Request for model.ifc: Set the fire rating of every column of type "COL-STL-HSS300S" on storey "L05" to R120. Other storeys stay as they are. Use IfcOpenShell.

First a look at what the model holds.

```python
import ifcopenshell
import ifcopenshell.util.element

model = ifcopenshell.open("model.ifc")
print(model.schema)
storey = next(s for s in model.by_type("IfcBuildingStorey") if s.Name == "L05")
columns = [e for e in ifcopenshell.util.element.get_decomposition(storey) if e.is_a("IfcColumn")]
seen = {}
for e in columns:
    element_type = ifcopenshell.util.element.get_type(e)
    key = (element_type.Name if element_type != e and element_type else None, ifcopenshell.util.element.get_pset(e, "Pset_ColumnCommon", "FireRating"))
    seen[key] = seen.get(key, 0) + 1
for (name, value), count in sorted(seen.items(), key=str):
    print(count, "x", name, "|", value)
```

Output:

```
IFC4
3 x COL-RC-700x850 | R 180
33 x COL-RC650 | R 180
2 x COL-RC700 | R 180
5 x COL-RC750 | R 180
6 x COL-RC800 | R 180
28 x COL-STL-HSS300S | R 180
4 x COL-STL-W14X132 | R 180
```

```python
import ifcopenshell
import ifcopenshell.api.pset
import ifcopenshell.util.element

model = ifcopenshell.open("model.ifc")

storey = next(s for s in model.by_type("IfcBuildingStorey") if s.Name == "L05")
columns = [e for e in ifcopenshell.util.element.get_decomposition(storey) if e.is_a("IfcColumn")]

count = 0
for e in columns:
    element_type = ifcopenshell.util.element.get_type(e)
    if element_type in (None, e) or element_type.Name != "COL-STL-HSS300S":
        continue
    # add_pset returns the element's existing set when there is one.
    pset = ifcopenshell.api.pset.add_pset(model, product=e, name="Pset_ColumnCommon")
    ifcopenshell.api.pset.edit_pset(model, pset=pset, properties={"FireRating": "R120"})
    count += 1

print(count, "columns updated")

model.write("model_updated.ifc")
```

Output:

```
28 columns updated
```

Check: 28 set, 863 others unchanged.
